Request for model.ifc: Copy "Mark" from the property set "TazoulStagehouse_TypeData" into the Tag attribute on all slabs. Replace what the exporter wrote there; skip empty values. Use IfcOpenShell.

First a look at what the model holds.

```python
import ifcopenshell
import ifcopenshell.util.element

model = ifcopenshell.open("model.ifc")
print(model.schema)
slabs = model.by_type("IfcSlab")
print(len(slabs), "slabs")
for e in slabs[:8]:
    source = ifcopenshell.util.element.get_pset(e, "TazoulStagehouse_TypeData", "Mark")
    target = e.Tag
    print(e.id(), repr(source), repr(target), sep=" | ")
```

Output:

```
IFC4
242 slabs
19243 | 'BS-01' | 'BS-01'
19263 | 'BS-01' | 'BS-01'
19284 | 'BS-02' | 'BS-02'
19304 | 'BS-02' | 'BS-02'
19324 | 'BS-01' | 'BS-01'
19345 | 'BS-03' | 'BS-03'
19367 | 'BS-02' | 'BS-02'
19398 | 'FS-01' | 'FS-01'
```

```python
import ifcopenshell
import ifcopenshell.util.element

model = ifcopenshell.open("model.ifc")

count = 0
for e in model.by_type("IfcSlab"):
    value = ifcopenshell.util.element.get_pset(e, "TazoulStagehouse_TypeData", "Mark")
    current = e.Tag
    if not value or not value.strip() or current == value:
        continue
    e.Tag = value
    count += 1

print(count, "slabs updated")

model.write("model-out.ifc")
```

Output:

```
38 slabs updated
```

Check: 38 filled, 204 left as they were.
